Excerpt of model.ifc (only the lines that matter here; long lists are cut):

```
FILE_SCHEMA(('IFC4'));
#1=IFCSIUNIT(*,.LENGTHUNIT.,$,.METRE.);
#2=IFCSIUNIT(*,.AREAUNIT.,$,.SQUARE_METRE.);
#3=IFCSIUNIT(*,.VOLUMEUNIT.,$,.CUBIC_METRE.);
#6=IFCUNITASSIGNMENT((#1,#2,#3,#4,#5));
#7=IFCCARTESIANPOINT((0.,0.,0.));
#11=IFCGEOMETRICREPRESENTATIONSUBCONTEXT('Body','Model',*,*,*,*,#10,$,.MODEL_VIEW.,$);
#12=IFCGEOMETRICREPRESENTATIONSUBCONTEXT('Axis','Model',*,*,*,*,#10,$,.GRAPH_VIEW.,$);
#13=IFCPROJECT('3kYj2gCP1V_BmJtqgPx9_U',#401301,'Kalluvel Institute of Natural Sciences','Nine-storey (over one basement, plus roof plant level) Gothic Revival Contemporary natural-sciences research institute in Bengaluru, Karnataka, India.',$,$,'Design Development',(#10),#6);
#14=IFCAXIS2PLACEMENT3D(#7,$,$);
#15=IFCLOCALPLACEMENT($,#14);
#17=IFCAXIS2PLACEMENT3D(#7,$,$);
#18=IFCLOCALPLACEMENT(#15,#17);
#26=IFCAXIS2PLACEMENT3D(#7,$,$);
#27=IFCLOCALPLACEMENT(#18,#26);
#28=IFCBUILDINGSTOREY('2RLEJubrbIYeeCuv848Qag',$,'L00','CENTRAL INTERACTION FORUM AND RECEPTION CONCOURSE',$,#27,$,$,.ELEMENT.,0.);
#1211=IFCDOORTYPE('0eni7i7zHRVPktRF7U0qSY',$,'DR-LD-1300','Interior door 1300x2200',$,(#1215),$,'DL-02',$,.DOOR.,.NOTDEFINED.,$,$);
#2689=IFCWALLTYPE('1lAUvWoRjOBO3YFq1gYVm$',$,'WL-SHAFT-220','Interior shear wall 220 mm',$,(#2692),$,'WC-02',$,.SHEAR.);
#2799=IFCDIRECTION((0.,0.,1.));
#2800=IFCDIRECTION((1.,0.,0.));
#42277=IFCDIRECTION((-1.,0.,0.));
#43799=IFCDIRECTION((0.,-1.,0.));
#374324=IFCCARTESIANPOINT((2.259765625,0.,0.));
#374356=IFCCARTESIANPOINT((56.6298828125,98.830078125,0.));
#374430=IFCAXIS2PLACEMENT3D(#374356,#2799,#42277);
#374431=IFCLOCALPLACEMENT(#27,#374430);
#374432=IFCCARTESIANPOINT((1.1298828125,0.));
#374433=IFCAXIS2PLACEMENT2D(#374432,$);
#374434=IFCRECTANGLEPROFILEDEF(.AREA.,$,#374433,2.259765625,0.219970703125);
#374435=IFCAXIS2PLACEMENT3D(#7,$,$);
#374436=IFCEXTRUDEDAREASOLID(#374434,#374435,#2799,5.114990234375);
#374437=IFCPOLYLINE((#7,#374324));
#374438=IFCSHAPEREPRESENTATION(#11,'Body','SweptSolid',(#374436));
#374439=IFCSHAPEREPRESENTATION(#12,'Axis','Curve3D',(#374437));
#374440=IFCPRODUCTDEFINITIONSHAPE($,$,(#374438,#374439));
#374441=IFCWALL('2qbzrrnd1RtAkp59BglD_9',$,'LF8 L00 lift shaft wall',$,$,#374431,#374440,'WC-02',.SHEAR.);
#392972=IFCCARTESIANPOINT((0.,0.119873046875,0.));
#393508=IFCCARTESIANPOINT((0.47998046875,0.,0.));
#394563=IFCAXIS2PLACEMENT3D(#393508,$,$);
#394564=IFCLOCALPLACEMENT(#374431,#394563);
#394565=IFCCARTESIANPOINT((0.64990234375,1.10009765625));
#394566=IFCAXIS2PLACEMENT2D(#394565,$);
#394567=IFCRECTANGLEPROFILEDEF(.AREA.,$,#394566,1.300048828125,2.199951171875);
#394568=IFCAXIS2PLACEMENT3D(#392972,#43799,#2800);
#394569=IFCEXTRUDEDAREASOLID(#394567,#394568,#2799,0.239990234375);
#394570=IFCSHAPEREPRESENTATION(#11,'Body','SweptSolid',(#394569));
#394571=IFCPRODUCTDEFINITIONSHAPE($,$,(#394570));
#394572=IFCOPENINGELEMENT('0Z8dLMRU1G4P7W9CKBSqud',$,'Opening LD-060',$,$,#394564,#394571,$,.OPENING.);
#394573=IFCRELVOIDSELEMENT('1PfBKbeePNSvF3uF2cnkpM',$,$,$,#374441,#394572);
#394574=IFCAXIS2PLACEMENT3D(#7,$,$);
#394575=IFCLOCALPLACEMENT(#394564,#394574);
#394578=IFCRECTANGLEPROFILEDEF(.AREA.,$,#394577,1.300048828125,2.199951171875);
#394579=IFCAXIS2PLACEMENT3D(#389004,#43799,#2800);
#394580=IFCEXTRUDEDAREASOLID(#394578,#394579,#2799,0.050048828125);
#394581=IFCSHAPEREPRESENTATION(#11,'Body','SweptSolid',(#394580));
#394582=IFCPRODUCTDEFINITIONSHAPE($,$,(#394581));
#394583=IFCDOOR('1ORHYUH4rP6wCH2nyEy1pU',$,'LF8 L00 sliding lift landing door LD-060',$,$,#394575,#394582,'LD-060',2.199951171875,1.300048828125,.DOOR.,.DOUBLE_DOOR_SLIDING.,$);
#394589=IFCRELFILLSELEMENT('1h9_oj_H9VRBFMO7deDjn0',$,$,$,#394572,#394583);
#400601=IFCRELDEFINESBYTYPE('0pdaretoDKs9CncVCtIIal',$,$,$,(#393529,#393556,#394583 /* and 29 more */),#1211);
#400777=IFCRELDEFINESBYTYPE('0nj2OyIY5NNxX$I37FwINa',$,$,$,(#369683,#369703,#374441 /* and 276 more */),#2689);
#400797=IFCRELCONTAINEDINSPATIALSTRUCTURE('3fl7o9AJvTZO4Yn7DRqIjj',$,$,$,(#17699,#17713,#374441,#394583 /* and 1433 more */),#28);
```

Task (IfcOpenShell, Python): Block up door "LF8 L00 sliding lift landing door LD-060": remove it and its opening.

```python
import ifcopenshell
import ifcopenshell.api.feature
import ifcopenshell.api.root
import ifcopenshell.geom
import ifcopenshell.util.shape

model = ifcopenshell.open("model.ifc")
settings = ifcopenshell.geom.settings()


def volume(element):
    """Net volume in cubic metres, openings subtracted."""
    shape = ifcopenshell.geom.create_shape(settings, element)
    return ifcopenshell.util.shape.get_volume(shape.geometry)


door = model.by_guid("1ORHYUH4rP6wCH2nyEy1pU")
opening = door.FillsVoids[0].RelatingOpeningElement
wall = opening.VoidsElements[0].RelatingBuildingElement
before = volume(wall)

ifcopenshell.api.root.remove_product(model, product=door)
ifcopenshell.api.feature.remove_feature(model, feature=opening)

after = volume(wall)

print(f"wall volume {before:.3f} -> {after:.3f} m3")

model.write("model_edited.ifc")
```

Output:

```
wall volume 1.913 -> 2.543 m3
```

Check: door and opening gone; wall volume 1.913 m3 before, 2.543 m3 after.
